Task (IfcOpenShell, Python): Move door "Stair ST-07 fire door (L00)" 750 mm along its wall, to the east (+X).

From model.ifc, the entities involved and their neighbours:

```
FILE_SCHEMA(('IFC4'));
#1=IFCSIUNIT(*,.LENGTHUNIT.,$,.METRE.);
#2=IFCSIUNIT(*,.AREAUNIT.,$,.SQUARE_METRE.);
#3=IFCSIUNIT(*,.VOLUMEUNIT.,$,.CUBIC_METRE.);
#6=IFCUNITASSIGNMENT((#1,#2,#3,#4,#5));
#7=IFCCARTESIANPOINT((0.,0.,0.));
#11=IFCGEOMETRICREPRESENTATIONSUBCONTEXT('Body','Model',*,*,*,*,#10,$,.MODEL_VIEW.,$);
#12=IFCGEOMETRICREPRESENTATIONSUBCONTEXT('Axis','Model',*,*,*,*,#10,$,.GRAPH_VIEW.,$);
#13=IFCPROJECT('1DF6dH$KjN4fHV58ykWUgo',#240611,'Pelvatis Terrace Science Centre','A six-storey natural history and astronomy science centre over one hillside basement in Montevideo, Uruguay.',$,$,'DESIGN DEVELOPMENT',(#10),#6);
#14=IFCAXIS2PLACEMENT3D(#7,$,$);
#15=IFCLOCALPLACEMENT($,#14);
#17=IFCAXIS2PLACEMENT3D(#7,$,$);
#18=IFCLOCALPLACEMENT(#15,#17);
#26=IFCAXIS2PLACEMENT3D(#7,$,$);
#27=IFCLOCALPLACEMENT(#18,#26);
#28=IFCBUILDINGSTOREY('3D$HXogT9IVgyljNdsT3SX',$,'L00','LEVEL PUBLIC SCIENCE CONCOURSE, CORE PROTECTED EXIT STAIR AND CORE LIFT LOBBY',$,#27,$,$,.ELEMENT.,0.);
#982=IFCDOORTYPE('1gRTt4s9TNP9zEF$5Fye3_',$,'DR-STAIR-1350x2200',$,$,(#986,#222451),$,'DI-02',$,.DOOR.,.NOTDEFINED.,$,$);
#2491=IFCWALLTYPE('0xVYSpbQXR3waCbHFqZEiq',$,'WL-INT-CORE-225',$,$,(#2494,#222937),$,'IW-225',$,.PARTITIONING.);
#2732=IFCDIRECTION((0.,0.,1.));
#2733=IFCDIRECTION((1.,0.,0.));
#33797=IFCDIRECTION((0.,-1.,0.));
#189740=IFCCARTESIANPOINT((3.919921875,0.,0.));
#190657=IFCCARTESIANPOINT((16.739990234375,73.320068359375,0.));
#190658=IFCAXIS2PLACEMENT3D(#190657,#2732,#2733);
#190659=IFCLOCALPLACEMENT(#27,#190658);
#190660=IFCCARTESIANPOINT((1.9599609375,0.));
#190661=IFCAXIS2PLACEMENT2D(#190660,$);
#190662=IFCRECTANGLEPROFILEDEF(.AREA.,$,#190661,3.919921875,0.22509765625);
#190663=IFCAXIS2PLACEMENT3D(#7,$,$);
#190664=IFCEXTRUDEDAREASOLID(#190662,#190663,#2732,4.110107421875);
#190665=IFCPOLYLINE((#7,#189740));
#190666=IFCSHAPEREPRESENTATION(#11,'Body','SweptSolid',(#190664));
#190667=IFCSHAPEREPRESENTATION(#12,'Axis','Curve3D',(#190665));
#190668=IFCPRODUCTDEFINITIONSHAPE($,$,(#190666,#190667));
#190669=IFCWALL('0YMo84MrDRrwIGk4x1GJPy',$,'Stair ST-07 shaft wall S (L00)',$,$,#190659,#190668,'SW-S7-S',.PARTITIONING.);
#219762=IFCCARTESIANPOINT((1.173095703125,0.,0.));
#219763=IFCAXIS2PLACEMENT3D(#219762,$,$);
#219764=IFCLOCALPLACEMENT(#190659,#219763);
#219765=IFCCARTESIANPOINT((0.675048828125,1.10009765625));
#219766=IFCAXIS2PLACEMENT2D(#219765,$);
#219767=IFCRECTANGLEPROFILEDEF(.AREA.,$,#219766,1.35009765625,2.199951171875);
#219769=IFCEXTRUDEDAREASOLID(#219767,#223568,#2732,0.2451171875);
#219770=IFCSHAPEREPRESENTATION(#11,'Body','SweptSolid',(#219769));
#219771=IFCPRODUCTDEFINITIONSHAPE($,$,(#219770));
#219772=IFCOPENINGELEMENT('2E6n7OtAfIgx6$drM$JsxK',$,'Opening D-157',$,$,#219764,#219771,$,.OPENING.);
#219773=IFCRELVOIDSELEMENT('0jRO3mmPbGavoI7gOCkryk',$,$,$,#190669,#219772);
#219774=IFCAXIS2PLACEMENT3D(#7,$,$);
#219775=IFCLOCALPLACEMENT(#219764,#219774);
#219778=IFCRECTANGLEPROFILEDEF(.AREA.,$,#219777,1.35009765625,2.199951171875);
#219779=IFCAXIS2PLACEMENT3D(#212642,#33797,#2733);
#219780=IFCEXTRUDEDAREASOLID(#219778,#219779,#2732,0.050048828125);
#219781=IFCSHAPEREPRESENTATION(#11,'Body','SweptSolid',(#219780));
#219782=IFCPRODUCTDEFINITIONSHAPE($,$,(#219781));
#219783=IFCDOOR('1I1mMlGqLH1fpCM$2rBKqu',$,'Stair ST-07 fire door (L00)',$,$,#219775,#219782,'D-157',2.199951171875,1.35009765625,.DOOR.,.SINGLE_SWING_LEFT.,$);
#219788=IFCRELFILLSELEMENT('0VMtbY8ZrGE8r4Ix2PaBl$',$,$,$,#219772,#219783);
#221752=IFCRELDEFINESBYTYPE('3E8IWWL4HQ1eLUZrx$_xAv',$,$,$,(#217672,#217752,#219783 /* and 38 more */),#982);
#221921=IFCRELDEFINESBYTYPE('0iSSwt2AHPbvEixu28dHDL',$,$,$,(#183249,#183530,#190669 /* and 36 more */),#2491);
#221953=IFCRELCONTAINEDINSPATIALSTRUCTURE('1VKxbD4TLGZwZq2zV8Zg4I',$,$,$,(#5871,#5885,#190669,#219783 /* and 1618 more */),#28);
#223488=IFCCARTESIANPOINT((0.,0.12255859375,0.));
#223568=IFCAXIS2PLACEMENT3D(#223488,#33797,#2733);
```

```python
import ifcopenshell
import ifcopenshell.api.geometry
import ifcopenshell.util.placement

model = ifcopenshell.open("model.ifc")

door = model.by_guid("1I1mMlGqLH1fpCM$2rBKqu")
opening = door.FillsVoids[0].RelatingOpeningElement
wall = opening.VoidsElements[0].RelatingBuildingElement

wall_matrix = ifcopenshell.util.placement.get_local_placement(wall.ObjectPlacement)
shift = wall_matrix[:3, 0] * 0.75
before = ifcopenshell.util.placement.get_local_placement(door.ObjectPlacement)[:3, 3].copy()

# The door is placed relative to its opening, so it follows when the opening moves.
matrix = ifcopenshell.util.placement.get_local_placement(opening.ObjectPlacement)
matrix[:3, 3] += shift
ifcopenshell.api.geometry.edit_object_placement(
    model, product=opening, matrix=matrix, is_si=False, should_transform_children=True
)

after = ifcopenshell.util.placement.get_local_placement(door.ObjectPlacement)[:3, 3]
print("door moved by", (after - before).round(3) + 0.0)

model.write("model_updated.ifc")
```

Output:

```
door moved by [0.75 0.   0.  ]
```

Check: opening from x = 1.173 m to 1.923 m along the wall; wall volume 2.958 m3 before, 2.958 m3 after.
